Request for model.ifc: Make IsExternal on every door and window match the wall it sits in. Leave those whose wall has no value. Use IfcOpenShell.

First a look at what the model holds.

```python
import ifcopenshell
import ifcopenshell.util.element

model = ifcopenshell.open("model.ifc")
print(model.schema)
seen = {}
for e in model.by_type("IfcDoor") + model.by_type("IfcWindow"):
    if not e.FillsVoids:
        continue
    host = e.FillsVoids[0].RelatingOpeningElement.VoidsElements[0].RelatingBuildingElement
    own = ifcopenshell.util.element.get_pset(e, f"Pset_{e.is_a()[3:].removesuffix('StandardCase')}Common", "IsExternal")
    wall = ifcopenshell.util.element.get_pset(host, "Pset_WallCommon", "IsExternal")
    seen[e.is_a(), own, wall] = seen.get((e.is_a(), own, wall), 0) + 1
for (cls, own, wall), count in sorted(seen.items(), key=str):
    print(count, cls, "IsExternal:", own, "| host wall:", wall)
```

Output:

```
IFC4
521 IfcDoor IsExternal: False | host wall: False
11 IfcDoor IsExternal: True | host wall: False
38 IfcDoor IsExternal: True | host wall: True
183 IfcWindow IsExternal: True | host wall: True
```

```python
import ifcopenshell
import ifcopenshell.api.pset
import ifcopenshell.util.element

model = ifcopenshell.open("model.ifc")

count = 0
for ifc_class, pset_name in (("IfcDoor", "Pset_DoorCommon"), ("IfcWindow", "Pset_WindowCommon")):
    for e in model.by_type(ifc_class):
        if not e.FillsVoids:
            continue
        host = e.FillsVoids[0].RelatingOpeningElement.VoidsElements[0].RelatingBuildingElement
        external = ifcopenshell.util.element.get_pset(host, "Pset_WallCommon", "IsExternal")
        if external is None or ifcopenshell.util.element.get_pset(e, pset_name, "IsExternal") == external:
            continue
        pset = ifcopenshell.api.pset.add_pset(model, product=e, name=pset_name)
        ifcopenshell.api.pset.edit_pset(model, pset=pset, properties={"IsExternal": external})
        count += 1

print(count, "updated")

model.write("model_edited.ifc")
```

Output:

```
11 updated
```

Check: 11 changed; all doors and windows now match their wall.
